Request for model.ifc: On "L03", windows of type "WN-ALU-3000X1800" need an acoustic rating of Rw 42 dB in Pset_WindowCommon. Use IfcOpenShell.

First a look at what the model holds.

```python
import ifcopenshell
import ifcopenshell.util.element

model = ifcopenshell.open("model.ifc")
print(model.schema)
storey = next(s for s in model.by_type("IfcBuildingStorey") if s.Name == "L03")
windows = [e for e in ifcopenshell.util.element.get_decomposition(storey) if e.is_a("IfcWindow")]
seen = {}
for e in windows:
    element_type = ifcopenshell.util.element.get_type(e)
    key = (element_type.Name if element_type != e and element_type else None, ifcopenshell.util.element.get_pset(e, "Pset_WindowCommon", "AcousticRating"))
    seen[key] = seen.get(key, 0) + 1
for (name, value), count in sorted(seen.items(), key=str):
    print(count, "x", name, "|", value)
```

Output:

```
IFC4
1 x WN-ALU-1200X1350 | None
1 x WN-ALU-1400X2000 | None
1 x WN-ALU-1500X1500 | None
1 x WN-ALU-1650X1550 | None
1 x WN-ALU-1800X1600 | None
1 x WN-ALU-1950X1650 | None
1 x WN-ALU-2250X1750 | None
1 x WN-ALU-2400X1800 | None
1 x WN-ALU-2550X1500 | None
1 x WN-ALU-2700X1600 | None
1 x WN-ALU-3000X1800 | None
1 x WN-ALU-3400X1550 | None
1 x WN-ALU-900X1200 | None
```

```python
import ifcopenshell
import ifcopenshell.api.pset
import ifcopenshell.util.element

model = ifcopenshell.open("model.ifc")

storey = next(s for s in model.by_type("IfcBuildingStorey") if s.Name == "L03")
windows = [e for e in ifcopenshell.util.element.get_decomposition(storey) if e.is_a("IfcWindow")]

count = 0
for e in windows:
    element_type = ifcopenshell.util.element.get_type(e)
    if element_type in (None, e) or element_type.Name != "WN-ALU-3000X1800":
        continue
    # add_pset returns the element's existing set when there is one.
    pset = ifcopenshell.api.pset.add_pset(model, product=e, name="Pset_WindowCommon")
    ifcopenshell.api.pset.edit_pset(model, pset=pset, properties={"AcousticRating": "Rw 42 dB"})
    count += 1

print(count, "windows updated")

model.write("model-out.ifc")
```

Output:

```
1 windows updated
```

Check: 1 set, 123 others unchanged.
